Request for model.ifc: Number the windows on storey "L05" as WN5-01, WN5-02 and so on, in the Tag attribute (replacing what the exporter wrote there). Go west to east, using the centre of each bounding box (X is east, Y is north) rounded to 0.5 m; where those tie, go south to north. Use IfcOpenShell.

First a look at what the model holds.

```python
import ifcopenshell
import ifcopenshell.util.element
import ifcopenshell.util.placement

model = ifcopenshell.open("model.ifc")
print(model.schema)
storey = next(s for s in model.by_type("IfcBuildingStorey") if s.Name == "L05")
windows = [e for e in ifcopenshell.util.element.get_decomposition(storey) if e.is_a("IfcWindow")]
for e in sorted(windows, key=lambda e: e.id()):
    origin = ifcopenshell.util.placement.get_local_placement(e.ObjectPlacement)[:3, 3]
    print(e.id(), e.Tag, e.Name, origin.round(2) + 0.0, sep=" | ")
```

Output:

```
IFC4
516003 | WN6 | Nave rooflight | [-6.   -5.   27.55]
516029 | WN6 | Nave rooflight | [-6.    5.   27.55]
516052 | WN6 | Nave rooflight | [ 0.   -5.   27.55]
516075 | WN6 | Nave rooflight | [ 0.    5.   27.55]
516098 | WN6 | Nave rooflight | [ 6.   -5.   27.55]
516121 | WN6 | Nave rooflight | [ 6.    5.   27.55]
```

```python
import ifcopenshell
import ifcopenshell.geom
import ifcopenshell.util.element
import ifcopenshell.util.shape

model = ifcopenshell.open("model.ifc")
settings = ifcopenshell.geom.settings()
settings.set("use-world-coords", True)


def centre(element):
    shape = ifcopenshell.geom.create_shape(settings, element)
    return ifcopenshell.util.shape.get_bbox_centroid(shape.geometry)


storey = next(s for s in model.by_type("IfcBuildingStorey") if s.Name == "L05")
windows = [e for e in ifcopenshell.util.element.get_decomposition(storey) if e.is_a("IfcWindow")]

# Insertion points can sit at a corner or the storey origin, so sort by the geometry (in metres).
centres = {e: centre(e) for e in windows}
windows.sort(key=lambda e: (round(centres[e][0] / 0.5), centres[e][1]))

for i, e in enumerate(windows, start=1):
    number = f"WN5-{i:02d}"
    e.Tag = number
    print(e.id(), number)

model.write("model_edited.ifc")
```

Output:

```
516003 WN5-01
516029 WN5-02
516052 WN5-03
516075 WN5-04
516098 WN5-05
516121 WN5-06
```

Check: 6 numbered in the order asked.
